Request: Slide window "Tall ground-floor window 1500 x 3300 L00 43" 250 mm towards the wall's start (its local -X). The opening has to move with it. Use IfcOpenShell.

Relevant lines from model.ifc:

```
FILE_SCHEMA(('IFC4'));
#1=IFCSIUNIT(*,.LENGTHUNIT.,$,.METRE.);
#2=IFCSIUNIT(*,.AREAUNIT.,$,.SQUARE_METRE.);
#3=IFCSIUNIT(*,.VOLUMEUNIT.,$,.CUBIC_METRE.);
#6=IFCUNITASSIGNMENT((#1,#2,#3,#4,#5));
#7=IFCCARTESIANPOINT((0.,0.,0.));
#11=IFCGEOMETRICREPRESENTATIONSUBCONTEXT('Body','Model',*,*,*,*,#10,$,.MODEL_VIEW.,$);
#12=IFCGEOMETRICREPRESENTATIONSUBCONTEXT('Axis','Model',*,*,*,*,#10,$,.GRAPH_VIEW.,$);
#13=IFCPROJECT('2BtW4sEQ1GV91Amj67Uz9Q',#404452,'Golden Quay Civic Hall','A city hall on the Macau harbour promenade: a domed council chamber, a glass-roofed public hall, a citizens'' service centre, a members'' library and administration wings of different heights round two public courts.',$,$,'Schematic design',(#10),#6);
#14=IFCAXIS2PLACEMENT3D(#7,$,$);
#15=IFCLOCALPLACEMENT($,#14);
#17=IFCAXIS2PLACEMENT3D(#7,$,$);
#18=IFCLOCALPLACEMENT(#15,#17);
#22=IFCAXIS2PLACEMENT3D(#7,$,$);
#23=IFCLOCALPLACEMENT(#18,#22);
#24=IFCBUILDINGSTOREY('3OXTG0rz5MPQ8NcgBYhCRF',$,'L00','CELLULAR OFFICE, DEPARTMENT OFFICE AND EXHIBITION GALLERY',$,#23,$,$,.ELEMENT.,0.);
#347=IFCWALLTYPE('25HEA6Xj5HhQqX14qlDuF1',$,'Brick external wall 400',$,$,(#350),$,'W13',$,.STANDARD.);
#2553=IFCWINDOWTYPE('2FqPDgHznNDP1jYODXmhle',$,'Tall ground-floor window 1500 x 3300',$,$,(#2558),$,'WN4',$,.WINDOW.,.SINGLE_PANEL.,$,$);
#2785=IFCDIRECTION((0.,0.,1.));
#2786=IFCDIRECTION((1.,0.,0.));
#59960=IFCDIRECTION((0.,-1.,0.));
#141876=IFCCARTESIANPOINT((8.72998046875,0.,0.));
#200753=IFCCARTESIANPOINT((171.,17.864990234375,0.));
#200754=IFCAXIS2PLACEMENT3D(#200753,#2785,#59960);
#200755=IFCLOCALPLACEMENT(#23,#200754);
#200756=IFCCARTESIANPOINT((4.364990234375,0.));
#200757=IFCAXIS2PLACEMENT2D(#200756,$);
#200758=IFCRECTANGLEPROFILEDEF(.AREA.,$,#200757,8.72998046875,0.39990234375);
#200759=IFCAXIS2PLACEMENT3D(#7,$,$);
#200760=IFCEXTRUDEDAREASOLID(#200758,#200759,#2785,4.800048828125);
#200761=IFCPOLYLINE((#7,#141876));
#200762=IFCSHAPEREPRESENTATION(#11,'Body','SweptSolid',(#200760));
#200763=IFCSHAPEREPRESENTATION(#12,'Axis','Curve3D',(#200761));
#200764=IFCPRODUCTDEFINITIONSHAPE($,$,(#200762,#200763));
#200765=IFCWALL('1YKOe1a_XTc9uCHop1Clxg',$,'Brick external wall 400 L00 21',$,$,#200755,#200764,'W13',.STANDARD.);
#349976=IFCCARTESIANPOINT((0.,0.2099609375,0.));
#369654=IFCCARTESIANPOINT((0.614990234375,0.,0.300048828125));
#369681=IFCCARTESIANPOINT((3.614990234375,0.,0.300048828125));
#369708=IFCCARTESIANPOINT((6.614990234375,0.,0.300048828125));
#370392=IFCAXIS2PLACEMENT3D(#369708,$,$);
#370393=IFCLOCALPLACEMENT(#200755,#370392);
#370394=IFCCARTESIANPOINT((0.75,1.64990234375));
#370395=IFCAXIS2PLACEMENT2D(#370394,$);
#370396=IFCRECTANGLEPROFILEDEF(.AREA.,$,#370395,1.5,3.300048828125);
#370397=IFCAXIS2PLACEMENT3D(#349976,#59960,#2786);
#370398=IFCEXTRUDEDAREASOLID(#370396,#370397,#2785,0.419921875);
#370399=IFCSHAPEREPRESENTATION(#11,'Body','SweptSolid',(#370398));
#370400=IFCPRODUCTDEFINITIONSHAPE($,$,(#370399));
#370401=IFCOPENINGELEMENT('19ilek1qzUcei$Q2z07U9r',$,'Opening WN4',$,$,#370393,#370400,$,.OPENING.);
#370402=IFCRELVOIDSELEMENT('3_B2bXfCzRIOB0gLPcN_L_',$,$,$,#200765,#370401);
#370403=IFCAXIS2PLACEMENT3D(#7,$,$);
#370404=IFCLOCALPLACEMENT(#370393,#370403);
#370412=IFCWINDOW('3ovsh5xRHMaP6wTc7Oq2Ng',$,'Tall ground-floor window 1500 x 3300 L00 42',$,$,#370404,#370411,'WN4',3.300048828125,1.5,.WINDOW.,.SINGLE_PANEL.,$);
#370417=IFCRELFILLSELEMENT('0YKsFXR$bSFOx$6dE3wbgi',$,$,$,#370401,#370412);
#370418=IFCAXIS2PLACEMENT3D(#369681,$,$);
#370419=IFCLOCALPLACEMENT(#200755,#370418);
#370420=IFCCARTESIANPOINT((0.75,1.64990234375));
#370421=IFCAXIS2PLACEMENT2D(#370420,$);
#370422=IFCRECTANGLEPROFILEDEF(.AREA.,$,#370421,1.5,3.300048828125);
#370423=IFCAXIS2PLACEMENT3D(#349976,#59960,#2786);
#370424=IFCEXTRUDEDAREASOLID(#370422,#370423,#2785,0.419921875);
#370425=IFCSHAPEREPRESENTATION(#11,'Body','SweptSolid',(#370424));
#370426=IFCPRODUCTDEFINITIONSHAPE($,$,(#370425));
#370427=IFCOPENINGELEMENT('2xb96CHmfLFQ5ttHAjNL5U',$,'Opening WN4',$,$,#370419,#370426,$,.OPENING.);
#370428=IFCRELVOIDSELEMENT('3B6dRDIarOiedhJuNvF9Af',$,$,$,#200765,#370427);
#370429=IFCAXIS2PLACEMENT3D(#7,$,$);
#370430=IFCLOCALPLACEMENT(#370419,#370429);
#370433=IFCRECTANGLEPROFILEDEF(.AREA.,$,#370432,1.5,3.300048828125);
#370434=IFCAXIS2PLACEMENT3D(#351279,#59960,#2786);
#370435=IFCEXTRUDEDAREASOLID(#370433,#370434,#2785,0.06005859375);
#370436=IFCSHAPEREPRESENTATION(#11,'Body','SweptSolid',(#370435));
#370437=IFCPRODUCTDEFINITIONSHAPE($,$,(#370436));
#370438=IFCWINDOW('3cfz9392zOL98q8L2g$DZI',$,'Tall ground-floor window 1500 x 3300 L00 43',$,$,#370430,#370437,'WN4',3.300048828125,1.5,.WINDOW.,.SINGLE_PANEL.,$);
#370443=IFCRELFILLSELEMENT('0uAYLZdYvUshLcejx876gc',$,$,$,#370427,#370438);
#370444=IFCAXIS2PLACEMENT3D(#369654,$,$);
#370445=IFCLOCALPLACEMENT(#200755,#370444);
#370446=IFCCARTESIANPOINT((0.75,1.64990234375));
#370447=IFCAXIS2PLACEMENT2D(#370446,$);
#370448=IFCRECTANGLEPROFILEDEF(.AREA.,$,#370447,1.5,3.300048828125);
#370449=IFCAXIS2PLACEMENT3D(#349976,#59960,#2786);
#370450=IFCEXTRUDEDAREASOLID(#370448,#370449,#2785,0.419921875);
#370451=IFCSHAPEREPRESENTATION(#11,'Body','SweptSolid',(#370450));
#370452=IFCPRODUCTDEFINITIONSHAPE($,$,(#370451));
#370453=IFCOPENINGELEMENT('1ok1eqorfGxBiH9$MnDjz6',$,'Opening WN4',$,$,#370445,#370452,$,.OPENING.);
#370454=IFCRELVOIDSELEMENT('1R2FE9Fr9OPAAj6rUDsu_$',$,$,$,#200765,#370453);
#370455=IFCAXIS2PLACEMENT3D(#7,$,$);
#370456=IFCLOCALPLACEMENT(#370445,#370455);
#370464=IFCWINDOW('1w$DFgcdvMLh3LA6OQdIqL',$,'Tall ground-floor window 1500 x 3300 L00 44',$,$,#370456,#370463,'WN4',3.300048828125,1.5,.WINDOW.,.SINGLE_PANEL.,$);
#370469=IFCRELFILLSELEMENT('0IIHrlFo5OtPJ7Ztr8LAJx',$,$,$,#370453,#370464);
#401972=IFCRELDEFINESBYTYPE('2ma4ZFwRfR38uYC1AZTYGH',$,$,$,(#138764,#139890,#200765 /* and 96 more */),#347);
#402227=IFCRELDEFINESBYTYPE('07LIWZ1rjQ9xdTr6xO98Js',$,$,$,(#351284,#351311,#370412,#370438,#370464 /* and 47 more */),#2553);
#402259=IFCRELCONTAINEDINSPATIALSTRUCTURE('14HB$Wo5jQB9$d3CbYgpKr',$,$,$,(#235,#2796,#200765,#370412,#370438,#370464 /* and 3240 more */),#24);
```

```python
import ifcopenshell
import ifcopenshell.api.geometry
import ifcopenshell.util.placement
import ifcopenshell.util.unit

model = ifcopenshell.open("model.ifc")
unit_scale = ifcopenshell.util.unit.calculate_unit_scale(model)

window = model.by_guid("3cfz9392zOL98q8L2g$DZI")
opening = window.FillsVoids[0].RelatingOpeningElement
wall = opening.VoidsElements[0].RelatingBuildingElement

wall_matrix = ifcopenshell.util.placement.get_local_placement(wall.ObjectPlacement)
shift = wall_matrix[:3, 0] * -0.25 / unit_scale
before = ifcopenshell.util.placement.get_local_placement(window.ObjectPlacement)[:3, 3].copy()

# The window is placed relative to its opening, so it follows when the opening moves.
matrix = ifcopenshell.util.placement.get_local_placement(opening.ObjectPlacement)
matrix[:3, 3] += shift
ifcopenshell.api.geometry.edit_object_placement(
    model, product=opening, matrix=matrix, is_si=False, should_transform_children=True
)

after = ifcopenshell.util.placement.get_local_placement(window.ObjectPlacement)[:3, 3]
print("window moved by", (after - before).round(3) + 0.0)

model.write("model_updated.ifc")
```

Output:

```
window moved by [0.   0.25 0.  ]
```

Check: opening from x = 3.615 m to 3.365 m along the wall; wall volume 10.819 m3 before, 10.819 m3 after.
